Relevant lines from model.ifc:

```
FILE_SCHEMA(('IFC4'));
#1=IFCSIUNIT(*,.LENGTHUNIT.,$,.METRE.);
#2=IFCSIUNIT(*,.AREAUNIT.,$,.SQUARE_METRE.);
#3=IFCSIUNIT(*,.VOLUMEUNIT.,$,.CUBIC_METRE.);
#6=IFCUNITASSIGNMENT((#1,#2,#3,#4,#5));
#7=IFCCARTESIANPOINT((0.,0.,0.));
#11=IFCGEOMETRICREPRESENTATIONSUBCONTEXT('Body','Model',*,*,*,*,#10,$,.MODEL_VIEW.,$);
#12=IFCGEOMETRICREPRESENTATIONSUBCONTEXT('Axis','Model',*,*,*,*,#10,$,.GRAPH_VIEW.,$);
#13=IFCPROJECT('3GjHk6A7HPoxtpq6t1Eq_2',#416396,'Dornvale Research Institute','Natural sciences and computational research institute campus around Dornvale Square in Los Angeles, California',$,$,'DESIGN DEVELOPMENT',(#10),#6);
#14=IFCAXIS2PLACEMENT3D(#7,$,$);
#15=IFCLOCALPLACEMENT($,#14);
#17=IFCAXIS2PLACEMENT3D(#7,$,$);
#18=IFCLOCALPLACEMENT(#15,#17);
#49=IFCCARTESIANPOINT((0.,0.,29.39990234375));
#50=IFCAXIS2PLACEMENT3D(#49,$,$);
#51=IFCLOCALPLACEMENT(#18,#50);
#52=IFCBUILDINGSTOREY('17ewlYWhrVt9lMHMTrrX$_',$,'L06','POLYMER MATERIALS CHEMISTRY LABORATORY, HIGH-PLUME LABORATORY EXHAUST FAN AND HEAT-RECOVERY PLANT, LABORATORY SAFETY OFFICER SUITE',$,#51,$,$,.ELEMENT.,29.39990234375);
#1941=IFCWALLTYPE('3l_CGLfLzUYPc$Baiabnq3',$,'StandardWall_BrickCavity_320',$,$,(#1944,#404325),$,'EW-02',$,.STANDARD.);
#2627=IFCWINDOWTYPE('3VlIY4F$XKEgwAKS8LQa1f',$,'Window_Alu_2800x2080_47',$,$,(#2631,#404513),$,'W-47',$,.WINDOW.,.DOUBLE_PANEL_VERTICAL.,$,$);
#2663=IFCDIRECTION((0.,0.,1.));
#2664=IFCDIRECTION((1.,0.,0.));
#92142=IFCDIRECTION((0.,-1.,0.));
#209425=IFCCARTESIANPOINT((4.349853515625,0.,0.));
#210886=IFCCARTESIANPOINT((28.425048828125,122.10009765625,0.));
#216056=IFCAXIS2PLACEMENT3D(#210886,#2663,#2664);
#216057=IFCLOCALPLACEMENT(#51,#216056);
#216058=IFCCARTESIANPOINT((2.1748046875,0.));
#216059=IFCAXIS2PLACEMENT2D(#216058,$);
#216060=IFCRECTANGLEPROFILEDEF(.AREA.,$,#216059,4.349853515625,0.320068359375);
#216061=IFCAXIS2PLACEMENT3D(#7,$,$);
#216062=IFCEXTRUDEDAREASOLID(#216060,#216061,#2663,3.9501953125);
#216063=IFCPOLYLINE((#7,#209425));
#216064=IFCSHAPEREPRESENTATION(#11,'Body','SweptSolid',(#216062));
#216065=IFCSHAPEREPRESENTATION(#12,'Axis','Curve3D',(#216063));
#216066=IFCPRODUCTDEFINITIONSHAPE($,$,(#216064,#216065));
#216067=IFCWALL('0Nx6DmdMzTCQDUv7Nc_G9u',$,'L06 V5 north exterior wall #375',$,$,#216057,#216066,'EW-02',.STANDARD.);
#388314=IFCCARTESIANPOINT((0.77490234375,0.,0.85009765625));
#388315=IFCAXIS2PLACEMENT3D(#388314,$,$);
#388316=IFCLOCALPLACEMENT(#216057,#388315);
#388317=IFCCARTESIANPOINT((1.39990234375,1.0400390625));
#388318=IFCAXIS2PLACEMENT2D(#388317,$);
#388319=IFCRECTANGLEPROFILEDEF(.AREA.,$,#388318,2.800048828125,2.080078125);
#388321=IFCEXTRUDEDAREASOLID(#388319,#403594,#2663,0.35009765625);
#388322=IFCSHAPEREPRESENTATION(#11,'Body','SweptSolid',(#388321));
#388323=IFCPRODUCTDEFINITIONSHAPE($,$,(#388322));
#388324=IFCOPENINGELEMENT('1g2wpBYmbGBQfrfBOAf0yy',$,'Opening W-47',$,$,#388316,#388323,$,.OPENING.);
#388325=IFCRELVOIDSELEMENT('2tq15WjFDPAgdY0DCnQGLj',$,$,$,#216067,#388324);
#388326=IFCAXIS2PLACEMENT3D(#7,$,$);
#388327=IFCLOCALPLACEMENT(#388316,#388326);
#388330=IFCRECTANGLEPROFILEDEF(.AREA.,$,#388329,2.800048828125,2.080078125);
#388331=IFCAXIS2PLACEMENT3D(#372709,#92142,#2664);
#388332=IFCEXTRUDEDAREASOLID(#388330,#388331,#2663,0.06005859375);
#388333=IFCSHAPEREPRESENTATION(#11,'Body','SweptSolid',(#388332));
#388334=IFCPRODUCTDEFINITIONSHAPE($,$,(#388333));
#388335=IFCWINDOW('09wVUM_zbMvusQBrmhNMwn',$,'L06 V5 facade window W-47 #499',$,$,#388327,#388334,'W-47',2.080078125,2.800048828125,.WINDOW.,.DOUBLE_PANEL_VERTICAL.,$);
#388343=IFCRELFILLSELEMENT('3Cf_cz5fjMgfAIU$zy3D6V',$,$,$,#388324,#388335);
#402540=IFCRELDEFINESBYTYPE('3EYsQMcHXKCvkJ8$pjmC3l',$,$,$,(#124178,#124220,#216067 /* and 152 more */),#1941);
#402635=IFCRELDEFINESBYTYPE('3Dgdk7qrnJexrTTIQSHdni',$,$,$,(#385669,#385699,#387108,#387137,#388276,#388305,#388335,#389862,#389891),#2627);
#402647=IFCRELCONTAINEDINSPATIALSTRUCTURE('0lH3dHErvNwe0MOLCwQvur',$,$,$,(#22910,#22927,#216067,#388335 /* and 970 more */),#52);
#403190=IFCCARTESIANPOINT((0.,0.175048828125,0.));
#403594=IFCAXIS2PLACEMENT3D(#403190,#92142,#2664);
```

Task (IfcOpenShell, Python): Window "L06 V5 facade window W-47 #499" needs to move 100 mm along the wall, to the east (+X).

```python
import ifcopenshell
import ifcopenshell.api.geometry
import ifcopenshell.util.placement
import ifcopenshell.util.unit

model = ifcopenshell.open("model.ifc")
unit_scale = ifcopenshell.util.unit.calculate_unit_scale(model)

window = model.by_guid("09wVUM_zbMvusQBrmhNMwn")
opening = window.FillsVoids[0].RelatingOpeningElement
wall = opening.VoidsElements[0].RelatingBuildingElement

wall_matrix = ifcopenshell.util.placement.get_local_placement(wall.ObjectPlacement)
shift = wall_matrix[:3, 0] * 0.1 / unit_scale
before = ifcopenshell.util.placement.get_local_placement(window.ObjectPlacement)[:3, 3].copy()

# The window is placed relative to its opening, so it follows when the opening moves.
matrix = ifcopenshell.util.placement.get_local_placement(opening.ObjectPlacement)
matrix[:3, 3] += shift
ifcopenshell.api.geometry.edit_object_placement(
    model, product=opening, matrix=matrix, is_si=False, should_transform_children=True
)

after = ifcopenshell.util.placement.get_local_placement(window.ObjectPlacement)[:3, 3]
print("window moved by", (after - before).round(3) + 0.0)

model.write("model_edited.ifc")
```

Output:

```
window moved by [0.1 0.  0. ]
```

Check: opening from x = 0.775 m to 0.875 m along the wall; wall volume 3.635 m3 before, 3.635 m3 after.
